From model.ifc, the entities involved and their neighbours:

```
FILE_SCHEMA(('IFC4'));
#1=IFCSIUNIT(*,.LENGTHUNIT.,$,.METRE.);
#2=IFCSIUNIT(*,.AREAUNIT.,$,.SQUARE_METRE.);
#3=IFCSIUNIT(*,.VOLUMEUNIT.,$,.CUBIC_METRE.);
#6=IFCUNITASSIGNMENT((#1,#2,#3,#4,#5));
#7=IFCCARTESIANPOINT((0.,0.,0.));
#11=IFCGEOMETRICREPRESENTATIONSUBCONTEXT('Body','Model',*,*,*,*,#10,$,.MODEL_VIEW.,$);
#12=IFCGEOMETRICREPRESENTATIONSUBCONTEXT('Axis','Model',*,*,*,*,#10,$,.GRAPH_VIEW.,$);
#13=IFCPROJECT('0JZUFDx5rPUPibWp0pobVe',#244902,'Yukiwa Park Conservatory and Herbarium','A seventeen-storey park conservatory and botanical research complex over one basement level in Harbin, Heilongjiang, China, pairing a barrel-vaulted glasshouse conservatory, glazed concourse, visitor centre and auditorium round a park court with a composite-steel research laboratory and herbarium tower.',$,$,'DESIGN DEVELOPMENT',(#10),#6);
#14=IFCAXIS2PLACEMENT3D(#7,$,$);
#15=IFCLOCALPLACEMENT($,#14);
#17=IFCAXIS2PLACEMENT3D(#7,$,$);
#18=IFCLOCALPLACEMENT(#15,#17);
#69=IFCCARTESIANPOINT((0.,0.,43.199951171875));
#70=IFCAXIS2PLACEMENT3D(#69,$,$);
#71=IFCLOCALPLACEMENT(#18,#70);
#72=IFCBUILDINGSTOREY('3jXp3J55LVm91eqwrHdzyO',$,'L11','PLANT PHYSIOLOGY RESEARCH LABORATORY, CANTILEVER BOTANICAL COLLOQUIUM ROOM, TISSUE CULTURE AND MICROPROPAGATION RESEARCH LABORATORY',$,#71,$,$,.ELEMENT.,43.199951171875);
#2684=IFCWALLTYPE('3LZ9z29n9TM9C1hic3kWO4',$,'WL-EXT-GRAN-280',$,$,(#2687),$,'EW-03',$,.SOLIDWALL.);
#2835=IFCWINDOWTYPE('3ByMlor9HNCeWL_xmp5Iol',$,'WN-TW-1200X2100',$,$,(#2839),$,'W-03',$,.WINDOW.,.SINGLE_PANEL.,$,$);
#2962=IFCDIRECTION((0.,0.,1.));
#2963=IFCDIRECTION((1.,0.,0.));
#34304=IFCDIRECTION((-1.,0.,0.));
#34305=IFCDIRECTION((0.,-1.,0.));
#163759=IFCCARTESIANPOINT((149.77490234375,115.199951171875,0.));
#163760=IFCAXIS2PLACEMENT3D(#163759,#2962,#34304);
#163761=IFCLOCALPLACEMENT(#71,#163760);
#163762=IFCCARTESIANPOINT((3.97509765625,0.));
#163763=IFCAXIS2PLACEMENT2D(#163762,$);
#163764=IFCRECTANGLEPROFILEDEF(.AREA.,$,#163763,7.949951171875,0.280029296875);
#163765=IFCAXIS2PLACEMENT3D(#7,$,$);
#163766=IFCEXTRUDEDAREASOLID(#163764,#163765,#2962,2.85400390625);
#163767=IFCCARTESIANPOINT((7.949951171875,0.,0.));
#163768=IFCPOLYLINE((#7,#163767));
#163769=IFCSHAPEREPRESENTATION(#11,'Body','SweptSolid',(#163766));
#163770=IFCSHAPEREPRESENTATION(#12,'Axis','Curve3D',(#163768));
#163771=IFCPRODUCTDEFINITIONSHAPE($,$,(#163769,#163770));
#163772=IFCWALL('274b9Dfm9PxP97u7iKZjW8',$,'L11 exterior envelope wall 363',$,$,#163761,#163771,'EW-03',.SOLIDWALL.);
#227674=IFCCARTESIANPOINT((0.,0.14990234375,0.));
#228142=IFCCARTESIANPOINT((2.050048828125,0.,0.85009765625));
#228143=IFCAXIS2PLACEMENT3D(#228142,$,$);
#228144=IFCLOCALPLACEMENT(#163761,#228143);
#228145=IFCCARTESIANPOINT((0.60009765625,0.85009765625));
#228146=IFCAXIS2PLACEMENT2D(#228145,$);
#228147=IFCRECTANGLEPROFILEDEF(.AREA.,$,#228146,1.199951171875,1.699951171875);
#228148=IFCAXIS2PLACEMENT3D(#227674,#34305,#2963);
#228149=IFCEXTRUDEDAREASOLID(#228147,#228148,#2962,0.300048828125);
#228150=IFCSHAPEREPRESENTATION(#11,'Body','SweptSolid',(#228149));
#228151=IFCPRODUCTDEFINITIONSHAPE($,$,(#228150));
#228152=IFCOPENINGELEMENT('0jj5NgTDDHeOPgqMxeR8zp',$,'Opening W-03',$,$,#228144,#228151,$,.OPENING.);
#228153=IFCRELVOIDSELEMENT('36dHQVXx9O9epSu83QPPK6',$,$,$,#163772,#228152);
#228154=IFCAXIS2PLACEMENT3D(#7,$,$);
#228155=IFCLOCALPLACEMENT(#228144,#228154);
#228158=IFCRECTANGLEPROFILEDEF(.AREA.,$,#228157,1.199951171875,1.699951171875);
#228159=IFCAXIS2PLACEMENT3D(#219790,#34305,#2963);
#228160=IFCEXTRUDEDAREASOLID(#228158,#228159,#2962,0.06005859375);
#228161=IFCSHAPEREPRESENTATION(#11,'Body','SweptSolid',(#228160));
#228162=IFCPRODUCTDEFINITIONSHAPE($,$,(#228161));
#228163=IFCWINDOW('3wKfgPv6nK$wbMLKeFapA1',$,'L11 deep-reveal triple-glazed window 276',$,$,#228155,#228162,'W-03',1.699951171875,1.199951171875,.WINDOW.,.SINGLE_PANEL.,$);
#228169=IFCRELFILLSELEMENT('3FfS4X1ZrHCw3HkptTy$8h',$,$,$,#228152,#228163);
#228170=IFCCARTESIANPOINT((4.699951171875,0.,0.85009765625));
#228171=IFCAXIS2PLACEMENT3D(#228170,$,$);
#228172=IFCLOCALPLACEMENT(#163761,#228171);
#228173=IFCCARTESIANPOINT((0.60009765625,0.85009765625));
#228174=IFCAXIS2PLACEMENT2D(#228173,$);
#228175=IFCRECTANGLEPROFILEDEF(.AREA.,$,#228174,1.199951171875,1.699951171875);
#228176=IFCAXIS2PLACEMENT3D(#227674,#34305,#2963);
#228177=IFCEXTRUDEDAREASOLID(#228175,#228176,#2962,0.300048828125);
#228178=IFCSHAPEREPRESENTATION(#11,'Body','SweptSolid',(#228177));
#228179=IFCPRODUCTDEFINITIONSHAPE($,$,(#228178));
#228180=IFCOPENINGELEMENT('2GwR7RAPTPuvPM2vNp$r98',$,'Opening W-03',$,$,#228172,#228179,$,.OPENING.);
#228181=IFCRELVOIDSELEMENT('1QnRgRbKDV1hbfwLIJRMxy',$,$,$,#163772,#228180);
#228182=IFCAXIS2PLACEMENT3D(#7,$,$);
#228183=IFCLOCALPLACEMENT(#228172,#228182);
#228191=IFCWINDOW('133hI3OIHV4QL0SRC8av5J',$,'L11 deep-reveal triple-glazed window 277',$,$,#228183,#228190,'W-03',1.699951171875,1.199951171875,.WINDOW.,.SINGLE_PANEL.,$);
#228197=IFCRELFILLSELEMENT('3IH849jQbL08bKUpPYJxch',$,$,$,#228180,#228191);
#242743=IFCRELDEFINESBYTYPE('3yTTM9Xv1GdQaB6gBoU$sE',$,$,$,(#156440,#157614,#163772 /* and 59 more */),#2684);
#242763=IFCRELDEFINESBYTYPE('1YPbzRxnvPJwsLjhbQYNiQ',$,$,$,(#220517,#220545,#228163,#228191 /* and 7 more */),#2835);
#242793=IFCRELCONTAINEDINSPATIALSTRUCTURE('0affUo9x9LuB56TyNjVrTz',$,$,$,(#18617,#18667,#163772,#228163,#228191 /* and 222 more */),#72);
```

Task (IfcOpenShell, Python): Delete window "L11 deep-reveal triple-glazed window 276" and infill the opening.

```python
import ifcopenshell
import ifcopenshell.api.feature
import ifcopenshell.api.root
import ifcopenshell.geom
import ifcopenshell.util.shape

model = ifcopenshell.open("model.ifc")
settings = ifcopenshell.geom.settings()


def volume(element):
    """Net volume in cubic metres, openings subtracted."""
    shape = ifcopenshell.geom.create_shape(settings, element)
    return ifcopenshell.util.shape.get_volume(shape.geometry)


window = model.by_guid("3wKfgPv6nK$wbMLKeFapA1")
opening = window.FillsVoids[0].RelatingOpeningElement
wall = opening.VoidsElements[0].RelatingBuildingElement
before = volume(wall)

ifcopenshell.api.root.remove_product(model, product=window)
ifcopenshell.api.feature.remove_feature(model, feature=opening)

after = volume(wall)

print(f"wall volume {before:.3f} -> {after:.3f} m3")

model.write("model_v2.ifc")
```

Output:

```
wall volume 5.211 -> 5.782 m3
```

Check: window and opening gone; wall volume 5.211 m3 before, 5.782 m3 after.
